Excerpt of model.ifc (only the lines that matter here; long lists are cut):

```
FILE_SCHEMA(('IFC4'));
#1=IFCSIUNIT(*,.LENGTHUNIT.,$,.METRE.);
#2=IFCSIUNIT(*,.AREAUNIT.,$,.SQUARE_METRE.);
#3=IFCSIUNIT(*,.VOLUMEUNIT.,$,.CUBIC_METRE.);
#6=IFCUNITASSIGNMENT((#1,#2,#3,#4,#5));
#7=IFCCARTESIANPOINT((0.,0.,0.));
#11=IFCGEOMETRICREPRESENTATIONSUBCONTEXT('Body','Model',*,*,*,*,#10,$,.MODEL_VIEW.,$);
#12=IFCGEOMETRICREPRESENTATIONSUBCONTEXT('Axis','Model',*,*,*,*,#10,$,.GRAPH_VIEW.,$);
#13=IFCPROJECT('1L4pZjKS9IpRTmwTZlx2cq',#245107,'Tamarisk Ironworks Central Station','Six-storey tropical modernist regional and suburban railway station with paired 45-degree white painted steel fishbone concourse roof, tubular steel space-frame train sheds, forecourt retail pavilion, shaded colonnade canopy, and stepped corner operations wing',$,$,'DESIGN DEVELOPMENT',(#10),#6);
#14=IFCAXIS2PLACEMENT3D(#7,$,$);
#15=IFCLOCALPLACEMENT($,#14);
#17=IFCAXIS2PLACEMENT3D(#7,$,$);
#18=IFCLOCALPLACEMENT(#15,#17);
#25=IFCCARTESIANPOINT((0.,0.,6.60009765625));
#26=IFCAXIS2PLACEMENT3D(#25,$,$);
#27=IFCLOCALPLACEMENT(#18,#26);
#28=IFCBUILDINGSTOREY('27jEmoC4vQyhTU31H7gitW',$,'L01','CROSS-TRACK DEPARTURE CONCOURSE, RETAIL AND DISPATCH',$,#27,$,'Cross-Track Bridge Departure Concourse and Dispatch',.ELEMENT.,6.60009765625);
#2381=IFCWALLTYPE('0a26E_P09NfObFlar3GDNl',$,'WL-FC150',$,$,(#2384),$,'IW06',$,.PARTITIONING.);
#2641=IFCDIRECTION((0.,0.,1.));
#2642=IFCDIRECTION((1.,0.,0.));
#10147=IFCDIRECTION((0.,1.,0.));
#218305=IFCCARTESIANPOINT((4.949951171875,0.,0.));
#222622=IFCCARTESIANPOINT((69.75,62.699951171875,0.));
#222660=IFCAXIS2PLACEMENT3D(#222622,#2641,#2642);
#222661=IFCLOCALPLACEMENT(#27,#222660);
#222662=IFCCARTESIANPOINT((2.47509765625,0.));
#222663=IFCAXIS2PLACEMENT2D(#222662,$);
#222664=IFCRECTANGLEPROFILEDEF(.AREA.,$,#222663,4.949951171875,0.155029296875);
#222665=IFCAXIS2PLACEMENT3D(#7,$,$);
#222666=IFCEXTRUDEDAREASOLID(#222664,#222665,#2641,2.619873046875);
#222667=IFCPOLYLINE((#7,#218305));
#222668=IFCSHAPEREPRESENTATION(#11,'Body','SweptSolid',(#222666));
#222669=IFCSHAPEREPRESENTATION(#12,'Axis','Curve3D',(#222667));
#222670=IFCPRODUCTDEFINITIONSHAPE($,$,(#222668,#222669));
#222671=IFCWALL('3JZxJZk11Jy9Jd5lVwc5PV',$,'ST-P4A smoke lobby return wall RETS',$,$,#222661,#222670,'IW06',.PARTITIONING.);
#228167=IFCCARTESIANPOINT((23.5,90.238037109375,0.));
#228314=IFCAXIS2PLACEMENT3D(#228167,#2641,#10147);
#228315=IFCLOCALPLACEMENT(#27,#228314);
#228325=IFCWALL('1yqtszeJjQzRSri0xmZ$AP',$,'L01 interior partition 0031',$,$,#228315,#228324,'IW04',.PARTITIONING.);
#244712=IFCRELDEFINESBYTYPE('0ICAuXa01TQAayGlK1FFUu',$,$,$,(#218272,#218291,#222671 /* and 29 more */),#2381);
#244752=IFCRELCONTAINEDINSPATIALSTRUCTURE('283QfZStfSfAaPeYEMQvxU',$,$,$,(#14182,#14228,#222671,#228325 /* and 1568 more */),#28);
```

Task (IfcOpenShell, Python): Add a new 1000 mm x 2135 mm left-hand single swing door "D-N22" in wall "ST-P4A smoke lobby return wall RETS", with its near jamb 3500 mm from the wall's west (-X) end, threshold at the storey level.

```python
import numpy as np
import ifcopenshell
import ifcopenshell.api.feature
import ifcopenshell.api.geometry
import ifcopenshell.api.root
import ifcopenshell.api.spatial
import ifcopenshell.geom
import ifcopenshell.util.element
import ifcopenshell.util.placement
import ifcopenshell.util.representation
import ifcopenshell.util.shape
import ifcopenshell.util.unit

model = ifcopenshell.open("model.ifc")
unit_scale = ifcopenshell.util.unit.calculate_unit_scale(model)
settings = ifcopenshell.geom.settings()


def volume(element):
    """Net volume in cubic metres, openings subtracted."""
    shape = ifcopenshell.geom.create_shape(settings, element)
    return ifcopenshell.util.shape.get_volume(shape.geometry)


wall = model.by_guid("3JZxJZk11Jy9Jd5lVwc5PV")
storey = ifcopenshell.util.element.get_container(wall, ifc_class="IfcBuildingStorey")
context = ifcopenshell.util.representation.get_context(model, "Model", "Body", "MODEL_VIEW")
before = volume(wall)

width, height, from_end, sill = 1, 2.135, 3.5, 0.0  # metres

# The wall runs along its own X axis, and the end named is its -X end.
wall_shape = ifcopenshell.geom.create_shape(settings, wall)
x, y, z = ifcopenshell.util.shape.get_vertices(wall_shape.geometry).T
start = x.min() + from_end
face, thickness = float(y.min()), float(y.max() - y.min())
wall_matrix = ifcopenshell.util.placement.get_local_placement(wall.ObjectPlacement)
level = ifcopenshell.util.placement.get_local_placement(storey.ObjectPlacement)[2, 3]


def in_wall(x, y):
    """Placement at x, y metres in the wall's axes, at sill height."""
    matrix = wall_matrix.copy()
    matrix[:, 3] = wall_matrix @ np.array([x / unit_scale, y / unit_scale, 0.0, 1.0])
    matrix[2, 3] = level + sill / unit_scale
    return matrix


# Opening: a box that overshoots both wall faces by 50 mm.
opening = ifcopenshell.api.root.create_entity(model, ifc_class="IfcOpeningElement", predefined_type="OPENING")
box = ifcopenshell.api.geometry.add_wall_representation(
    model, context=context, length=width, height=height, thickness=thickness + 0.1
)
ifcopenshell.api.geometry.assign_representation(model, product=opening, representation=box)
ifcopenshell.api.geometry.edit_object_placement(model, product=opening, matrix=in_wall(start, face - 0.05), is_si=False)
ifcopenshell.api.feature.add_feature(model, feature=opening, element=wall)

door = ifcopenshell.api.root.create_entity(model, ifc_class="IfcDoor", name="D-N22", predefined_type="DOOR")
door.OverallWidth, door.OverallHeight = width / unit_scale, height / unit_scale
door.OperationType = "SINGLE_SWING_LEFT"
body = ifcopenshell.api.geometry.add_door_representation(
    model,
    context=context,
    overall_width=door.OverallWidth,
    overall_height=door.OverallHeight,
    operation_type="SINGLE_SWING_LEFT",
    lining_properties={"LiningDepth": thickness / unit_scale, "ThresholdDepth": thickness / unit_scale},
)
ifcopenshell.api.geometry.assign_representation(model, product=door, representation=body)
ifcopenshell.api.spatial.assign_container(model, products=[door], relating_structure=storey)
ifcopenshell.api.feature.add_filling(model, opening=opening, element=door)

# The lining spans the wall, so the door starts at the wall face.
ifcopenshell.api.geometry.edit_object_placement(model, product=door, matrix=in_wall(start, face), is_si=False)

after = volume(wall)

print(f"wall volume {before:.3f} -> {after:.3f} m3")

model.write("model_v2.ifc")
```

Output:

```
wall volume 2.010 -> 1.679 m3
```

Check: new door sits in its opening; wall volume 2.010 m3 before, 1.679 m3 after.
